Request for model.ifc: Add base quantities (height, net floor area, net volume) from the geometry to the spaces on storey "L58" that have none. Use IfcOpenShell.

First a look at what the model holds.

```python
import ifcopenshell
import ifcopenshell.util.element
import ifcopenshell.util.unit

model = ifcopenshell.open("model.ifc")
print(model.schema)
for unit_type in ("LENGTHUNIT", "AREAUNIT", "VOLUMEUNIT"):
    print(unit_type, ifcopenshell.util.unit.calculate_unit_scale(model, unit_type))
storey = next(s for s in model.by_type("IfcBuildingStorey") if s.Name == "L58")
spaces = [e for e in ifcopenshell.util.element.get_decomposition(storey) if e.is_a("IfcSpace")]
for e in sorted(spaces, key=lambda e: e.id()):
    print(e.id(), e.is_a(), e.Name, list(ifcopenshell.util.element.get_psets(e, qtos_only=True)), sep=" | ")
```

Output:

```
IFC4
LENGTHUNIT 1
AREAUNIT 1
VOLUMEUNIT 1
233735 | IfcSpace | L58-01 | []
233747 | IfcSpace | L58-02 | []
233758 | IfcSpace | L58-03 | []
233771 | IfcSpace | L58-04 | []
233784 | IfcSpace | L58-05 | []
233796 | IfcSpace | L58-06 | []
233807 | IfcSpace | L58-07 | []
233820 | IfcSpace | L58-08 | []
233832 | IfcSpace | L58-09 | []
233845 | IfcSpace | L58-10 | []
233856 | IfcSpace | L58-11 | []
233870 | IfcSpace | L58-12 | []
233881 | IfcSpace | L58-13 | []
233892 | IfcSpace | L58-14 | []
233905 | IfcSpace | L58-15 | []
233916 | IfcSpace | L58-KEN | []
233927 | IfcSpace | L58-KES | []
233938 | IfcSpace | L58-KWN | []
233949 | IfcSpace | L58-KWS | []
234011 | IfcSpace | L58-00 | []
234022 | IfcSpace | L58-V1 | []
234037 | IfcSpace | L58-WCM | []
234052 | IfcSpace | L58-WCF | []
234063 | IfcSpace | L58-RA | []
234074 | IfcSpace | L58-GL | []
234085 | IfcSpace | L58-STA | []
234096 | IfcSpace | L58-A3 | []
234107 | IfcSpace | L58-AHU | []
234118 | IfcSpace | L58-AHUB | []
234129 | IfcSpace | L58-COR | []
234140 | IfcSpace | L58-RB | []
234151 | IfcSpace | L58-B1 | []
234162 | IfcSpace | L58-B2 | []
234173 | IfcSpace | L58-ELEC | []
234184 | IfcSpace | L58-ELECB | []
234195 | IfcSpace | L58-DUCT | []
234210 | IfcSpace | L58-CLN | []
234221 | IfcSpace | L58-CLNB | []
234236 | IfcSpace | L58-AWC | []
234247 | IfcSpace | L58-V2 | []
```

```python
import ifcopenshell
import ifcopenshell.api.pset
import ifcopenshell.geom
import ifcopenshell.util.element
import ifcopenshell.util.shape
import ifcopenshell.util.unit

model = ifcopenshell.open("model.ifc")
unit_scale = ifcopenshell.util.unit.calculate_unit_scale(model)
area_scale = ifcopenshell.util.unit.calculate_unit_scale(model, "AREAUNIT")
volume_scale = ifcopenshell.util.unit.calculate_unit_scale(model, "VOLUMEUNIT")
settings = ifcopenshell.geom.settings()

storey = next(s for s in model.by_type("IfcBuildingStorey") if s.Name == "L58")
spaces = [e for e in ifcopenshell.util.element.get_decomposition(storey) if e.is_a("IfcSpace")]

for e in sorted(spaces, key=lambda e: e.id()):
    if ifcopenshell.util.element.get_psets(e, qtos_only=True, should_inherit=False):
        continue
    # Geometry comes back in metres, in the element's own axes.
    shape = ifcopenshell.geom.create_shape(settings, e)
    values = {
        "Height": ifcopenshell.util.shape.get_z(shape.geometry) / unit_scale,
        "NetFloorArea": ifcopenshell.util.shape.get_footprint_area(shape.geometry) / area_scale,
        "NetVolume": ifcopenshell.util.shape.get_volume(shape.geometry) / volume_scale,
    }
    qto = ifcopenshell.api.pset.add_qto(model, product=e, name="Qto_SpaceBaseQuantities")
    ifcopenshell.api.pset.edit_qto(model, qto=qto, properties=values)
    print(e.id(), {k: round(v, 3) for k, v in values.items()})

model.write("model_updated.ifc")
```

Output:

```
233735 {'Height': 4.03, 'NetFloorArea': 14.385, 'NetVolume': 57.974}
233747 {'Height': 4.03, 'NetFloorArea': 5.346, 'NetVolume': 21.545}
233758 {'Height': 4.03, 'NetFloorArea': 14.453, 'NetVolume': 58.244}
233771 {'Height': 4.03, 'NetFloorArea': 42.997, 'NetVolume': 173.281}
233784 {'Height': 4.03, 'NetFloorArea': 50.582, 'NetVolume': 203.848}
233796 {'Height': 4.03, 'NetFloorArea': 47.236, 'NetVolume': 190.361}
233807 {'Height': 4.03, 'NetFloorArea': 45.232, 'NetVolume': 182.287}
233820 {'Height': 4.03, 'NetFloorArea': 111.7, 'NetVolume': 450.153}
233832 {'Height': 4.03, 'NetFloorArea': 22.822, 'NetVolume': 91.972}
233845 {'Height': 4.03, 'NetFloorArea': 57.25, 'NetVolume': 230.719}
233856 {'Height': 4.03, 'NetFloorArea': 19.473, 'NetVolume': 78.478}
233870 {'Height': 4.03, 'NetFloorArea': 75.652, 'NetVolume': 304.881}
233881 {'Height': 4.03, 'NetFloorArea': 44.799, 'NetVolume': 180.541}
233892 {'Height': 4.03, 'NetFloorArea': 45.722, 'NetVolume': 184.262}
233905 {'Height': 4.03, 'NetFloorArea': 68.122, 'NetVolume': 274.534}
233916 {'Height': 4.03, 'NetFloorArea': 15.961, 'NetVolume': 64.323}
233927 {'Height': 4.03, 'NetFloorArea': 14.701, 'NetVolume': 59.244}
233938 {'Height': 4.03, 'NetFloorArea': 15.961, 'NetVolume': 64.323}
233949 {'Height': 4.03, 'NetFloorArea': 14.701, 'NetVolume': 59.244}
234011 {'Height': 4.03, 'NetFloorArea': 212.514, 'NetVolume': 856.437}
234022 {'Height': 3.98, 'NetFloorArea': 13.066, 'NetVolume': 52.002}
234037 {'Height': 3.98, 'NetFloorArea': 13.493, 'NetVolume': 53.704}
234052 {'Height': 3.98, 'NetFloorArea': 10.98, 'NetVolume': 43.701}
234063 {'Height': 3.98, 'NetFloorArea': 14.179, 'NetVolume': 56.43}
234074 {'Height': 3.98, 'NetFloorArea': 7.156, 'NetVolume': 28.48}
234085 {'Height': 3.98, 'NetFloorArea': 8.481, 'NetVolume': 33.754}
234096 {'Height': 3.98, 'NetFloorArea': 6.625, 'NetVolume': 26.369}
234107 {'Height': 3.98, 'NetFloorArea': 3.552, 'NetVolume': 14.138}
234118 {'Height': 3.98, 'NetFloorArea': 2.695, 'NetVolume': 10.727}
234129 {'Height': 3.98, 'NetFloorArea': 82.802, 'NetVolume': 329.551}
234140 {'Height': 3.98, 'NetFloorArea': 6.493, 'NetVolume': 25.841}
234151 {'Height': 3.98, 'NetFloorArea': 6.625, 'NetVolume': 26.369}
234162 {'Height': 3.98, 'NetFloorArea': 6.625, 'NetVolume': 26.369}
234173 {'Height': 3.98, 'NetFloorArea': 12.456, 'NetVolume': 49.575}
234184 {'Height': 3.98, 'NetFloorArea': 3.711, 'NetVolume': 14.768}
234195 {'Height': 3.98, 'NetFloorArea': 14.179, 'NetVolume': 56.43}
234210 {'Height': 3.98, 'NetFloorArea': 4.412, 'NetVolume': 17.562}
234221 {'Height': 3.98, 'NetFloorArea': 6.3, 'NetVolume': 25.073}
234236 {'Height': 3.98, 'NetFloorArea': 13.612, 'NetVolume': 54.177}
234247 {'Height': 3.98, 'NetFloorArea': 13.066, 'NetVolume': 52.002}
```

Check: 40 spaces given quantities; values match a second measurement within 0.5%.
